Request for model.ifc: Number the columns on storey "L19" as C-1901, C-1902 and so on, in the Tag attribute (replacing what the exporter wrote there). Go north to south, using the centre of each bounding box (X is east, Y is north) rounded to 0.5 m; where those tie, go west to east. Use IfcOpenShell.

First a look at what the model holds.

```python
import ifcopenshell
import ifcopenshell.util.element
import ifcopenshell.util.placement

model = ifcopenshell.open("model.ifc")
print(model.schema)
storey = next(s for s in model.by_type("IfcBuildingStorey") if s.Name == "L19")
columns = [e for e in ifcopenshell.util.element.get_decomposition(storey) if e.is_a("IfcColumn")]
for e in sorted(columns, key=lambda e: e.id()):
    origin = ifcopenshell.util.placement.get_local_placement(e.ObjectPlacement)[:3, 3]
    print(e.id(), e.Tag, e.Name, origin.round(2) + 0.0, sep=" | ")
```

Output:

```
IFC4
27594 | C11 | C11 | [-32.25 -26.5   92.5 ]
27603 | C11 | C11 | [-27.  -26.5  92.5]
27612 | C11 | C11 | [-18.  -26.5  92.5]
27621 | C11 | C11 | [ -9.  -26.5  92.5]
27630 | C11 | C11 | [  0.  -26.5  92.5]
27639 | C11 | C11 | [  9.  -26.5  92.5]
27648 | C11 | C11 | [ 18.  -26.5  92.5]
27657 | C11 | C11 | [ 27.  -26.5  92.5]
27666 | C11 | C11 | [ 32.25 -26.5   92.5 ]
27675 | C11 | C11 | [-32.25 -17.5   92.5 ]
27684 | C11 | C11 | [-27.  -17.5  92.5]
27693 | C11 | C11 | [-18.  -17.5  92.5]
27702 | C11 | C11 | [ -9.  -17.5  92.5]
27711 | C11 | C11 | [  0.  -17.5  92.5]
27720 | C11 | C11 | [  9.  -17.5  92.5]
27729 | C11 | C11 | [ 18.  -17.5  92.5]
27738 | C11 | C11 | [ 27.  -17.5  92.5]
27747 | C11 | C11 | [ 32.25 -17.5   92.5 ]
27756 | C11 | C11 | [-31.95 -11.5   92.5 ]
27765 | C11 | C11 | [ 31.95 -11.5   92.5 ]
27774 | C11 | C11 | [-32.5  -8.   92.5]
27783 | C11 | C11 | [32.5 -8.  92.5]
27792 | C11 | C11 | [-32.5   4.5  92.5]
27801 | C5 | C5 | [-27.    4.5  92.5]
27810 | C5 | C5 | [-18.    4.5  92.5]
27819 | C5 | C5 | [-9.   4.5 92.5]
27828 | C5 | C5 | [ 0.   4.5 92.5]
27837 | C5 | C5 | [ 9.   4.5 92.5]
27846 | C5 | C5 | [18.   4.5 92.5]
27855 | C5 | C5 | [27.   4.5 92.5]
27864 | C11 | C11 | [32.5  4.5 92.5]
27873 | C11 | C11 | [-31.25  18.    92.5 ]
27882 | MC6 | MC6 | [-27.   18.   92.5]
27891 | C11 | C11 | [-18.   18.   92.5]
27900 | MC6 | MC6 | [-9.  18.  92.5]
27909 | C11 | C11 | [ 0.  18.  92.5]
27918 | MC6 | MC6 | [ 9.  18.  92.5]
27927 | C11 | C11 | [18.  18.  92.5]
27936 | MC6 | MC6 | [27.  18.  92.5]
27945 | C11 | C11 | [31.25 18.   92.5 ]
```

```python
import ifcopenshell
import ifcopenshell.geom
import ifcopenshell.util.element
import ifcopenshell.util.shape

model = ifcopenshell.open("model.ifc")
settings = ifcopenshell.geom.settings()
settings.set("use-world-coords", True)


def centre(element):
    shape = ifcopenshell.geom.create_shape(settings, element)
    return ifcopenshell.util.shape.get_bbox_centroid(shape.geometry)


storey = next(s for s in model.by_type("IfcBuildingStorey") if s.Name == "L19")
columns = [e for e in ifcopenshell.util.element.get_decomposition(storey) if e.is_a("IfcColumn")]

# Insertion points can sit at a corner or the storey origin, so sort by the geometry (in metres).
centres = {e: centre(e) for e in columns}
columns.sort(key=lambda e: (-round(centres[e][1] / 0.5), centres[e][0]))

for i, e in enumerate(columns, start=1):
    number = f"C-19{i:02d}"
    e.Tag = number
    print(e.id(), number)

model.write("model_rev.ifc")
```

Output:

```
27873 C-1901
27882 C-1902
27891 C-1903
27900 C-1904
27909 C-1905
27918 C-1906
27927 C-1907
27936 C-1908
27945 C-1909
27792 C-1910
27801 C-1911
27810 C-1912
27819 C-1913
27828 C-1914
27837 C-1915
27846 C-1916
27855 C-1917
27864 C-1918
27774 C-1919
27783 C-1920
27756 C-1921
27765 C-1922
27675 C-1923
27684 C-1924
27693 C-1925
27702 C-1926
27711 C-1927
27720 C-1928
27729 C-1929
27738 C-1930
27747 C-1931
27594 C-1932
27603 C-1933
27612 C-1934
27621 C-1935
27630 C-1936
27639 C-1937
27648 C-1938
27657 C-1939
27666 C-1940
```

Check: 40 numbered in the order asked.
